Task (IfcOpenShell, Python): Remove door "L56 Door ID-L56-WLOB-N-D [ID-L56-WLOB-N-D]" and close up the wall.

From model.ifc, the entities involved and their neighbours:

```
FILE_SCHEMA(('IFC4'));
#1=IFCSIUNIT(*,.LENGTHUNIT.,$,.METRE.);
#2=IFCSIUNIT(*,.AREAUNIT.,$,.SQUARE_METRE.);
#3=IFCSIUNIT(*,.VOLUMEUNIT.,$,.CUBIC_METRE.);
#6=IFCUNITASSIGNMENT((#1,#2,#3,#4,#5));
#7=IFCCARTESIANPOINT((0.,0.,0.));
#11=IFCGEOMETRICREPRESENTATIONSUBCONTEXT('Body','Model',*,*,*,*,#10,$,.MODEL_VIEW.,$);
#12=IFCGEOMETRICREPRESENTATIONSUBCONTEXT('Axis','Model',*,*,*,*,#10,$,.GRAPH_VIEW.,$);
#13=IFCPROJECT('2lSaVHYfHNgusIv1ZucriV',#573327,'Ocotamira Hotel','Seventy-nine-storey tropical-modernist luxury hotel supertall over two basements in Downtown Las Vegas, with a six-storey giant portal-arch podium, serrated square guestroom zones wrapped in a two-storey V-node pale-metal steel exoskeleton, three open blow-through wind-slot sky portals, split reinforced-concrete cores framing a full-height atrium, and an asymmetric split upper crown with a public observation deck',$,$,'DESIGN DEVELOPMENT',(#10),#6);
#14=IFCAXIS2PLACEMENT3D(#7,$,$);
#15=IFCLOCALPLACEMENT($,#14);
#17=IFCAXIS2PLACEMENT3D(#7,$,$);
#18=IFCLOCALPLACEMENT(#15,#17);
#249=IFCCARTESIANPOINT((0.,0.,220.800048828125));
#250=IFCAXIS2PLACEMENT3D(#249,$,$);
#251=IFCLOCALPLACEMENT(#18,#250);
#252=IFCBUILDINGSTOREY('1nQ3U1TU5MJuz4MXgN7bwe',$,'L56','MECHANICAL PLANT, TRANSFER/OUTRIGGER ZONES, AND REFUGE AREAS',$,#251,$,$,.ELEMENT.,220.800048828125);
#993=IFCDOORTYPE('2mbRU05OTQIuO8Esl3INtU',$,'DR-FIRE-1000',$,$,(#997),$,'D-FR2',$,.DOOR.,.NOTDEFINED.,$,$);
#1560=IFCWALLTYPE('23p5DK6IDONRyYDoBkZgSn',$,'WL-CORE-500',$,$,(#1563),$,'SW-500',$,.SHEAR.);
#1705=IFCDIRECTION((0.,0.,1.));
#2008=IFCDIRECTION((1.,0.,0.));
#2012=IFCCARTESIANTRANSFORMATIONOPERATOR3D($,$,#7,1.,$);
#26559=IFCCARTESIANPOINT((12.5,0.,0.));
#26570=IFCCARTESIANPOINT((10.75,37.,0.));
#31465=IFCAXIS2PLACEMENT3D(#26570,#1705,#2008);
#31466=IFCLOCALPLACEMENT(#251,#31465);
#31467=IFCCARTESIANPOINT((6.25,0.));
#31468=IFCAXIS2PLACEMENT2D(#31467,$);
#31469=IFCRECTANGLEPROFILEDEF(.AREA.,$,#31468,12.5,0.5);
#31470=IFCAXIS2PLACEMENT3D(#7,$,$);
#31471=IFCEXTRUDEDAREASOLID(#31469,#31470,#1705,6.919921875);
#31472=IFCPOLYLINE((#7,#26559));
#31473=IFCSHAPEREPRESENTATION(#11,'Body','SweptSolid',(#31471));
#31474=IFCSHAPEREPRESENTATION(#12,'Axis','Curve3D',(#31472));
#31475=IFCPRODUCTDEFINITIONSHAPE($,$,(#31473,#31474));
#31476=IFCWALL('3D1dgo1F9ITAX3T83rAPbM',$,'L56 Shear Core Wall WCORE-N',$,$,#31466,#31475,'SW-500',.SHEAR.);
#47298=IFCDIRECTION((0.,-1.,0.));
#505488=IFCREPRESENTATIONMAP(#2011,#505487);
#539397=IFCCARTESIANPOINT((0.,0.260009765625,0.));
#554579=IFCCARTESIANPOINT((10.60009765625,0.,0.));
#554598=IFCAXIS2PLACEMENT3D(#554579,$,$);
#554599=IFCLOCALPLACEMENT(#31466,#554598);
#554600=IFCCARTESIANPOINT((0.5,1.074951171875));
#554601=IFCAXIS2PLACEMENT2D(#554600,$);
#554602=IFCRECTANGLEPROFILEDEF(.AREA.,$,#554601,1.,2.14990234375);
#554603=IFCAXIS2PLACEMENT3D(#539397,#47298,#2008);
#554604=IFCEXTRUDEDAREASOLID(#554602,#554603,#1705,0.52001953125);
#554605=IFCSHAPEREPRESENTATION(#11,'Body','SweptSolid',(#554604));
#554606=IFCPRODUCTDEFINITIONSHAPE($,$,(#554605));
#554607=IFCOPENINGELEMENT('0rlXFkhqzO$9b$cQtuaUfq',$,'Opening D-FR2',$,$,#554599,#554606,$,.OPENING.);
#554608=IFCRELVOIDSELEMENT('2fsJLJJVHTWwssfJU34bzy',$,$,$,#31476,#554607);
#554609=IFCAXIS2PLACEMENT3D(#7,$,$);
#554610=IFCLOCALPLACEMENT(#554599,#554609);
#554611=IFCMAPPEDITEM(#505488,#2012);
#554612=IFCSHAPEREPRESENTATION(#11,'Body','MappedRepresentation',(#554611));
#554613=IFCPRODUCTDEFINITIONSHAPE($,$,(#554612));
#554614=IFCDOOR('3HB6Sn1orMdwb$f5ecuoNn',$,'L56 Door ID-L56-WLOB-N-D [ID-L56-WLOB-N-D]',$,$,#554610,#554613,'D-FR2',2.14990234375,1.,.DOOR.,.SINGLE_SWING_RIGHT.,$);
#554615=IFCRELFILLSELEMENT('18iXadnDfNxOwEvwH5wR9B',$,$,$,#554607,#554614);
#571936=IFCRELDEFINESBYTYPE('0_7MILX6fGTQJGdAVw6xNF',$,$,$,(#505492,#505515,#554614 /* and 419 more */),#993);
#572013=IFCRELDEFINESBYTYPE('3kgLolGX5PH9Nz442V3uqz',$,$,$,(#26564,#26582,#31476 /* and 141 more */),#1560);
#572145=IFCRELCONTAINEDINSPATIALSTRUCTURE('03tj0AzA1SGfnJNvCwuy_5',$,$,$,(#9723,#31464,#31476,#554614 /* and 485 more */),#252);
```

```python
import ifcopenshell
import ifcopenshell.api.feature
import ifcopenshell.api.root
import ifcopenshell.geom
import ifcopenshell.util.shape

model = ifcopenshell.open("model.ifc")
settings = ifcopenshell.geom.settings()


def volume(element):
    """Net volume in cubic metres, openings subtracted."""
    shape = ifcopenshell.geom.create_shape(settings, element)
    return ifcopenshell.util.shape.get_volume(shape.geometry)


door = model.by_id(554614)
opening = door.FillsVoids[0].RelatingOpeningElement
wall = opening.VoidsElements[0].RelatingBuildingElement
before = volume(wall)

ifcopenshell.api.root.remove_product(model, product=door)
ifcopenshell.api.feature.remove_feature(model, feature=opening)

after = volume(wall)

print(f"wall volume {before:.3f} -> {after:.3f} m3")

model.write("model_rev.ifc")
```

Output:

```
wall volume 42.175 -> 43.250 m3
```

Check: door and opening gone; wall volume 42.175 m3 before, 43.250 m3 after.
